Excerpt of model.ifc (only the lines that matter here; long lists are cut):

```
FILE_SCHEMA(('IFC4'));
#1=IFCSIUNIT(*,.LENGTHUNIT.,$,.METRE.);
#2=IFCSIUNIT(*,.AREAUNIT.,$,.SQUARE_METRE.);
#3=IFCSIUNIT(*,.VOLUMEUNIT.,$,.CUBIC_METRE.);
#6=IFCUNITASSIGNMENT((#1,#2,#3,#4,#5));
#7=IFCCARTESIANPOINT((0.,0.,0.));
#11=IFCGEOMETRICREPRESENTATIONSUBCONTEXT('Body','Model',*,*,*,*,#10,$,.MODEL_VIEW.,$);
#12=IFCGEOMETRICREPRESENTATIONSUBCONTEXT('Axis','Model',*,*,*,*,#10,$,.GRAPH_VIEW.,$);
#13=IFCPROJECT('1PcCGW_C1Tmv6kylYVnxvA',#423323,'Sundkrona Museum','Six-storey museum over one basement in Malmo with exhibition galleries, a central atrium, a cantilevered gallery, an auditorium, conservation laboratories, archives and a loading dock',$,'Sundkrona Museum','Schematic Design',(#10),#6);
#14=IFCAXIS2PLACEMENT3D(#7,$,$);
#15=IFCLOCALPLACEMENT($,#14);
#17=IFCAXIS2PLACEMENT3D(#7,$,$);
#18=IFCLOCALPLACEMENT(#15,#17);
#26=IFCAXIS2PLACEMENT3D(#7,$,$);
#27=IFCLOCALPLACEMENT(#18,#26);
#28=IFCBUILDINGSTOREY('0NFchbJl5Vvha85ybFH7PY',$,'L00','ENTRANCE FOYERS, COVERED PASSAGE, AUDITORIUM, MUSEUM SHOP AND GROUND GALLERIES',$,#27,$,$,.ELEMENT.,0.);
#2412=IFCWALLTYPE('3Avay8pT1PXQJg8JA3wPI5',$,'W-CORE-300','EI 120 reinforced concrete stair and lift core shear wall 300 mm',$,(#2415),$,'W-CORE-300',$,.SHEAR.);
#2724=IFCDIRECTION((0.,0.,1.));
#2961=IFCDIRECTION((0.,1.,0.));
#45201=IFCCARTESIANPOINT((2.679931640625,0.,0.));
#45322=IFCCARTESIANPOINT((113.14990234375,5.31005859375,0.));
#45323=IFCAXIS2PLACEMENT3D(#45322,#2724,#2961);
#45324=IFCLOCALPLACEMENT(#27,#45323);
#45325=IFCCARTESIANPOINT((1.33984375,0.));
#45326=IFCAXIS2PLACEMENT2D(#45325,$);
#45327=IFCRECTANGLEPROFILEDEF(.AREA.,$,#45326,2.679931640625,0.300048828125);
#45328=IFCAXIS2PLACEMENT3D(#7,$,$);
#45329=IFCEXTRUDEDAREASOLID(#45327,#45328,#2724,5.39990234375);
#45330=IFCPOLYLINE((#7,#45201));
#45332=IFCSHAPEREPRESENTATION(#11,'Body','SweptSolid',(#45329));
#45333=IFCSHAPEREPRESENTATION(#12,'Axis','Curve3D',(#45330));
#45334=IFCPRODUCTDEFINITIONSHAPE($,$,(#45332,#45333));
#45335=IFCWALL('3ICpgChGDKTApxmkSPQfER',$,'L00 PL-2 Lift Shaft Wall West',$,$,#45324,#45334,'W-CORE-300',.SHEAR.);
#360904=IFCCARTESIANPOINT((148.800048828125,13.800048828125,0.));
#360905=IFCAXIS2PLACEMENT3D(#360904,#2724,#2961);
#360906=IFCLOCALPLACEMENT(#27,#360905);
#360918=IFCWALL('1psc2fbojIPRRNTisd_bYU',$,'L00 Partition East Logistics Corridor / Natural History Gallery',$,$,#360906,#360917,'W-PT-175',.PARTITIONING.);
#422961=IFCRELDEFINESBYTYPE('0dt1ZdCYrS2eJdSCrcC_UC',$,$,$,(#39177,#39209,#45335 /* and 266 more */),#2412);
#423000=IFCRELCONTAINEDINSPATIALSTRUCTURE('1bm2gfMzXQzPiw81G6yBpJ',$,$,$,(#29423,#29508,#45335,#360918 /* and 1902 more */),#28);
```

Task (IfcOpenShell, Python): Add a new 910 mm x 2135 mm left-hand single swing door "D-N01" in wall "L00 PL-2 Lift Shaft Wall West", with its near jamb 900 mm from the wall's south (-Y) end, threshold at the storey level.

```python
import numpy as np
import ifcopenshell
import ifcopenshell.api.feature
import ifcopenshell.api.geometry
import ifcopenshell.api.root
import ifcopenshell.api.spatial
import ifcopenshell.geom
import ifcopenshell.util.element
import ifcopenshell.util.placement
import ifcopenshell.util.representation
import ifcopenshell.util.shape
import ifcopenshell.util.unit

model = ifcopenshell.open("model.ifc")
unit_scale = ifcopenshell.util.unit.calculate_unit_scale(model)
settings = ifcopenshell.geom.settings()


def volume(element):
    """Net volume in cubic metres, openings subtracted."""
    shape = ifcopenshell.geom.create_shape(settings, element)
    return ifcopenshell.util.shape.get_volume(shape.geometry)


wall = model.by_guid("3ICpgChGDKTApxmkSPQfER")
storey = ifcopenshell.util.element.get_container(wall, ifc_class="IfcBuildingStorey")
context = ifcopenshell.util.representation.get_context(model, "Model", "Body", "MODEL_VIEW")
before = volume(wall)

width, height, from_end, sill = 0.91, 2.135, 0.9, 0.0  # metres

# The wall runs along its own X axis, and the end named is its -X end.
wall_shape = ifcopenshell.geom.create_shape(settings, wall)
x, y, z = ifcopenshell.util.shape.get_vertices(wall_shape.geometry).T
start = x.min() + from_end
face, thickness = float(y.min()), float(y.max() - y.min())
wall_matrix = ifcopenshell.util.placement.get_local_placement(wall.ObjectPlacement)
level = ifcopenshell.util.placement.get_local_placement(storey.ObjectPlacement)[2, 3]


def in_wall(x, y):
    """Placement at x, y metres in the wall's axes, at sill height."""
    matrix = wall_matrix.copy()
    matrix[:, 3] = wall_matrix @ np.array([x / unit_scale, y / unit_scale, 0.0, 1.0])
    matrix[2, 3] = level + sill / unit_scale
    return matrix


# Opening: a box that overshoots both wall faces by 50 mm.
opening = ifcopenshell.api.root.create_entity(model, ifc_class="IfcOpeningElement", predefined_type="OPENING")
box = ifcopenshell.api.geometry.add_wall_representation(
    model, context=context, length=width, height=height, thickness=thickness + 0.1
)
ifcopenshell.api.geometry.assign_representation(model, product=opening, representation=box)
ifcopenshell.api.geometry.edit_object_placement(model, product=opening, matrix=in_wall(start, face - 0.05), is_si=False)
ifcopenshell.api.feature.add_feature(model, feature=opening, element=wall)

door = ifcopenshell.api.root.create_entity(model, ifc_class="IfcDoor", name="D-N01", predefined_type="DOOR")
door.OverallWidth, door.OverallHeight = width / unit_scale, height / unit_scale
door.OperationType = "SINGLE_SWING_LEFT"
body = ifcopenshell.api.geometry.add_door_representation(
    model,
    context=context,
    overall_width=door.OverallWidth,
    overall_height=door.OverallHeight,
    operation_type="SINGLE_SWING_LEFT",
    lining_properties={"LiningDepth": thickness / unit_scale, "ThresholdDepth": thickness / unit_scale},
)
ifcopenshell.api.geometry.assign_representation(model, product=door, representation=body)
ifcopenshell.api.spatial.assign_container(model, products=[door], relating_structure=storey)
ifcopenshell.api.feature.add_filling(model, opening=opening, element=door)

# The lining spans the wall, so the door starts at the wall face.
ifcopenshell.api.geometry.edit_object_placement(model, product=door, matrix=in_wall(start, face), is_si=False)

after = volume(wall)

print(f"wall volume {before:.3f} -> {after:.3f} m3")

model.write("model_edited.ifc")
```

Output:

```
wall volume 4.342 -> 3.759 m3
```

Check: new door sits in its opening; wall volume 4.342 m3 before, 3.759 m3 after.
